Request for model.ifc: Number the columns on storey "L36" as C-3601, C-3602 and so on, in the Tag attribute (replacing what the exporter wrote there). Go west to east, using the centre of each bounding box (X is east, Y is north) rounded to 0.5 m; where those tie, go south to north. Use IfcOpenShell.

First a look at what the model holds.

```python
import ifcopenshell
import ifcopenshell.util.element
import ifcopenshell.util.placement

model = ifcopenshell.open("model.ifc")
print(model.schema)
storey = next(s for s in model.by_type("IfcBuildingStorey") if s.Name == "L36")
columns = [e for e in ifcopenshell.util.element.get_decomposition(storey) if e.is_a("IfcColumn")]
for e in sorted(columns, key=lambda e: e.id()):
    origin = ifcopenshell.util.placement.get_local_placement(e.ObjectPlacement)[:3, 3]
    print(e.id(), e.Tag, e.Name, origin.round(2) + 0.0, sep=" | ")
```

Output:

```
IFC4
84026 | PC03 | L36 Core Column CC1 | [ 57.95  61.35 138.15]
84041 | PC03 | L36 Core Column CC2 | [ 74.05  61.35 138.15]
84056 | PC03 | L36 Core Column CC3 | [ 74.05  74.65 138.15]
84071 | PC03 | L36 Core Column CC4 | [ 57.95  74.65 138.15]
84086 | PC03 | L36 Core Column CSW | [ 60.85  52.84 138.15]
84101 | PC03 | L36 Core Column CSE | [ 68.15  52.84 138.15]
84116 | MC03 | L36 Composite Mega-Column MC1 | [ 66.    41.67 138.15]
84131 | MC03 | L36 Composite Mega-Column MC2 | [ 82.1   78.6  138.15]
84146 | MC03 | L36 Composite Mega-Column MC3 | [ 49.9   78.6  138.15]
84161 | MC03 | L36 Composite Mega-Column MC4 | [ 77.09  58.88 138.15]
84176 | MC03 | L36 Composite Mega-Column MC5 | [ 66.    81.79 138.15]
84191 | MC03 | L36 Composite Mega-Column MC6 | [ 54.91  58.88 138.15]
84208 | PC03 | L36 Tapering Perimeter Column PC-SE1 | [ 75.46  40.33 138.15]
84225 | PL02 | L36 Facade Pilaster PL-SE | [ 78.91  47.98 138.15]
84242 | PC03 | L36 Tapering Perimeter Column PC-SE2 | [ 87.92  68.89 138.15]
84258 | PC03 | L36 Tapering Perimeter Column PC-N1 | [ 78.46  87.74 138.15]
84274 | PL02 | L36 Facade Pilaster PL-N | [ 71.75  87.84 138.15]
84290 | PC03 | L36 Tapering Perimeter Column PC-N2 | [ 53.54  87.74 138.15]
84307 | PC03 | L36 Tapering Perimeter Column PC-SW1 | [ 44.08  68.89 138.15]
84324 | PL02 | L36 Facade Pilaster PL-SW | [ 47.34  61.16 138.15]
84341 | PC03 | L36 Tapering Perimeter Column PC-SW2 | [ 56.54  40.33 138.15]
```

```python
import ifcopenshell
import ifcopenshell.geom
import ifcopenshell.util.element
import ifcopenshell.util.shape

model = ifcopenshell.open("model.ifc")
settings = ifcopenshell.geom.settings()
settings.set("use-world-coords", True)


def centre(element):
    shape = ifcopenshell.geom.create_shape(settings, element)
    return ifcopenshell.util.shape.get_bbox_centroid(shape.geometry)


storey = next(s for s in model.by_type("IfcBuildingStorey") if s.Name == "L36")
columns = [e for e in ifcopenshell.util.element.get_decomposition(storey) if e.is_a("IfcColumn")]

# Insertion points can sit at a corner or the storey origin, so sort by the geometry (in metres).
centres = {e: centre(e) for e in columns}
columns.sort(key=lambda e: (round(centres[e][0] / 0.5), centres[e][1]))

for i, e in enumerate(columns, start=1):
    number = f"C-36{i:02d}"
    e.Tag = number
    print(e.id(), number)

model.write("model_rev.ifc")
```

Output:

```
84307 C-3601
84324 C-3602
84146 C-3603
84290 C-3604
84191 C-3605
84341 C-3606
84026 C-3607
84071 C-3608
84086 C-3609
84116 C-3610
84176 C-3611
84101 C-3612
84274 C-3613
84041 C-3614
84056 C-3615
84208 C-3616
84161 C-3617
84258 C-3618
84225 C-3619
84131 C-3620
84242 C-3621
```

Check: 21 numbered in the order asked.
